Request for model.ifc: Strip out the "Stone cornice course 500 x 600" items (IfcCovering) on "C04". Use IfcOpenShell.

First a look at what the model holds.

```python
import ifcopenshell
import ifcopenshell.util.element

model = ifcopenshell.open("model.ifc")
print(model.schema)
storey = next(s for s in model.by_type("IfcBuildingStorey") if s.Name == "C04")
coverings = [e for e in ifcopenshell.util.element.get_decomposition(storey) if e.is_a("IfcCovering")]
seen = {}
for e in coverings:
    element_type = ifcopenshell.util.element.get_type(e)
    name = element_type.Name if element_type not in (None, e) else None
    seen[name] = seen.get(name, 0) + 1
for name, count in sorted(seen.items(), key=str):
    print(count, "x", name)
```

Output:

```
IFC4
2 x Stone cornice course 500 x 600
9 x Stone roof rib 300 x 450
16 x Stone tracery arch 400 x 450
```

```python
import ifcopenshell
import ifcopenshell.api.root
import ifcopenshell.util.element

model = ifcopenshell.open("model.ifc")

storey = next(s for s in model.by_type("IfcBuildingStorey") if s.Name == "C04")
coverings = [e for e in ifcopenshell.util.element.get_decomposition(storey) if e.is_a("IfcCovering")]
targets = [e for e in coverings if (t := ifcopenshell.util.element.get_type(e)) not in (None, e) and t.Name == "Stone cornice course 500 x 600"]

for e in targets:
    ifcopenshell.api.root.remove_product(model, product=e)
print(len(targets), "removed")

model.write("model_rev.ifc")
```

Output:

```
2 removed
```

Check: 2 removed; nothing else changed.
